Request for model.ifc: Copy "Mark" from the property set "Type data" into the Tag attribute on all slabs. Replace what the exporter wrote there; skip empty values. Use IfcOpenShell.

First a look at what the model holds.

```python
import ifcopenshell
import ifcopenshell.util.element

model = ifcopenshell.open("model.ifc")
print(model.schema)
slabs = model.by_type("IfcSlab")
print(len(slabs), "slabs")
for e in slabs[:8]:
    source = ifcopenshell.util.element.get_pset(e, "Type data", "Mark")
    target = e.Tag
    print(e.id(), repr(source), repr(target), sep=" | ")
```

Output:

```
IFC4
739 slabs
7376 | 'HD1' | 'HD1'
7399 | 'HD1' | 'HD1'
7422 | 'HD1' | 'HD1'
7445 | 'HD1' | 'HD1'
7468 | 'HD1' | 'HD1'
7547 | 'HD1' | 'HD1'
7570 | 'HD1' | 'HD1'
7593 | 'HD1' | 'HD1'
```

```python
import ifcopenshell
import ifcopenshell.util.element

model = ifcopenshell.open("model.ifc")

count = 0
for e in model.by_type("IfcSlab"):
    value = ifcopenshell.util.element.get_pset(e, "Type data", "Mark")
    current = e.Tag
    if not value or not value.strip() or current == value:
        continue
    e.Tag = value
    count += 1

print(count, "slabs updated")

model.write("model_edited.ifc")
```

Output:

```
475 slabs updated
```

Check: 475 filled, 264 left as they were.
